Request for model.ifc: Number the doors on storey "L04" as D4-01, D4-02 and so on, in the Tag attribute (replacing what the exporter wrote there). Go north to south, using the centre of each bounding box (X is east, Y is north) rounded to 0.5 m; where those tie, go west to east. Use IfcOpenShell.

First a look at what the model holds.

```python
import ifcopenshell
import ifcopenshell.util.element
import ifcopenshell.util.placement

model = ifcopenshell.open("model.ifc")
print(model.schema)
storey = next(s for s in model.by_type("IfcBuildingStorey") if s.Name == "L04")
doors = [e for e in ifcopenshell.util.element.get_decomposition(storey) if e.is_a("IfcDoor")]
for e in sorted(doors, key=lambda e: e.id()):
    origin = ifcopenshell.util.placement.get_local_placement(e.ObjectPlacement)[:3, 3]
    print(e.id(), e.Tag, e.Name, origin.round(2) + 0.0, sep=" | ")
```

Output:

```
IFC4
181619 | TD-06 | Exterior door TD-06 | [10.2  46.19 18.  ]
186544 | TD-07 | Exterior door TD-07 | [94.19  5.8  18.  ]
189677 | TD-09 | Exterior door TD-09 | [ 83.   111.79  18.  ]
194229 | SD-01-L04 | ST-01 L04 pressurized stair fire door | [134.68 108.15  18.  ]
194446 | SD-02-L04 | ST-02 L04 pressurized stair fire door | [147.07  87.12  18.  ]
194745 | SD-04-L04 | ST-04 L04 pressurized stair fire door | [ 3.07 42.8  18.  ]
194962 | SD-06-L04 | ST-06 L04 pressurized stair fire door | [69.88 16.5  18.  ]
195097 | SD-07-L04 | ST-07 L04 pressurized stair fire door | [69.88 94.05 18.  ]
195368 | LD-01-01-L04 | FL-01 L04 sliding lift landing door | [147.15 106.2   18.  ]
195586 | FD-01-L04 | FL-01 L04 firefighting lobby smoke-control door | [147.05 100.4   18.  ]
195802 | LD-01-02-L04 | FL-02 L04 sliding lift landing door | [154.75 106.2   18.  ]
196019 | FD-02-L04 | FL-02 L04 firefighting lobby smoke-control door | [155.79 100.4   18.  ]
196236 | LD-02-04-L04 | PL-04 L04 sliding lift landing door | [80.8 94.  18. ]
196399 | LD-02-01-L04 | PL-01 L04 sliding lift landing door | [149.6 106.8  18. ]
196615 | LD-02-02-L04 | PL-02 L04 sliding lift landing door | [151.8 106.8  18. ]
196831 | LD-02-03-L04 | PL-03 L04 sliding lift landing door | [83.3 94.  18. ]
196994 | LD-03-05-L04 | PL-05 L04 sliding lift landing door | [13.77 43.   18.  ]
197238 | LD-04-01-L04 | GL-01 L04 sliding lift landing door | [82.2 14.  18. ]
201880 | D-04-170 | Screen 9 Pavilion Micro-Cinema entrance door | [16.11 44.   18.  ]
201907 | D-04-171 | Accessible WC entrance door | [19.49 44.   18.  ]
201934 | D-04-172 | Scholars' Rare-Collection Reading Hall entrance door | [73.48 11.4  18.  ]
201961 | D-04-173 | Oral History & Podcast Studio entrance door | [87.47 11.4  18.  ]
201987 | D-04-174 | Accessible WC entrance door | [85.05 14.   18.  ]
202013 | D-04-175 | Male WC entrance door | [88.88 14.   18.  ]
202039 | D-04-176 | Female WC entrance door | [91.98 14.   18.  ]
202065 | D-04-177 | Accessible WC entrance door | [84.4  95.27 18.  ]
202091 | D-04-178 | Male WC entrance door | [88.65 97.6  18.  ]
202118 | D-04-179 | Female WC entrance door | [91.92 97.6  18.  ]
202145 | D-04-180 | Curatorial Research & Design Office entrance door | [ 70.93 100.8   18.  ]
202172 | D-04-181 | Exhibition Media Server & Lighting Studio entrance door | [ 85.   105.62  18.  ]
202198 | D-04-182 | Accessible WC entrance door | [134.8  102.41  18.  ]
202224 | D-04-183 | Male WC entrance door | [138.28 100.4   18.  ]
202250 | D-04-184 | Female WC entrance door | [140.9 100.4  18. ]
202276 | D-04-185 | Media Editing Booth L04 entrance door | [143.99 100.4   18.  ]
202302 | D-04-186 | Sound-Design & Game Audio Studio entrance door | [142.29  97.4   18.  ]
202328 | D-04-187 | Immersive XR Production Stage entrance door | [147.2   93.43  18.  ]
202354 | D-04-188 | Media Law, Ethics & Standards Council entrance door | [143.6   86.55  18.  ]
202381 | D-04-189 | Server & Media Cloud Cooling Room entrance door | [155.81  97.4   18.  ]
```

```python
import ifcopenshell
import ifcopenshell.geom
import ifcopenshell.util.element
import ifcopenshell.util.shape

model = ifcopenshell.open("model.ifc")
settings = ifcopenshell.geom.settings()
settings.set("use-world-coords", True)


def centre(element):
    shape = ifcopenshell.geom.create_shape(settings, element)
    return ifcopenshell.util.shape.get_bbox_centroid(shape.geometry)


storey = next(s for s in model.by_type("IfcBuildingStorey") if s.Name == "L04")
doors = [e for e in ifcopenshell.util.element.get_decomposition(storey) if e.is_a("IfcDoor")]

# Insertion points can sit at a corner or the storey origin, so sort by the geometry (in metres).
centres = {e: centre(e) for e in doors}
doors.sort(key=lambda e: (-round(centres[e][1] / 0.5), centres[e][0]))

for i, e in enumerate(doors, start=1):
    number = f"D4-{i:02d}"
    e.Tag = number
    print(e.id(), number)

model.write("model_rev.ifc")
```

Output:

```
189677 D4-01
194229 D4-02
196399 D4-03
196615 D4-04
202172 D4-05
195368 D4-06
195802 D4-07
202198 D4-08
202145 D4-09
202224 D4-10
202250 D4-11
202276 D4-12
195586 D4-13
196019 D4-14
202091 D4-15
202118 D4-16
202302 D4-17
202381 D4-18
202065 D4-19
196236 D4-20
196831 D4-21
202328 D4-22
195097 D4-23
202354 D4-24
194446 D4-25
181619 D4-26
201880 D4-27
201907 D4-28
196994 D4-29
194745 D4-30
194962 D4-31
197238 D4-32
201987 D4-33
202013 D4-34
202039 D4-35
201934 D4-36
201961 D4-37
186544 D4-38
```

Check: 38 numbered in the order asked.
